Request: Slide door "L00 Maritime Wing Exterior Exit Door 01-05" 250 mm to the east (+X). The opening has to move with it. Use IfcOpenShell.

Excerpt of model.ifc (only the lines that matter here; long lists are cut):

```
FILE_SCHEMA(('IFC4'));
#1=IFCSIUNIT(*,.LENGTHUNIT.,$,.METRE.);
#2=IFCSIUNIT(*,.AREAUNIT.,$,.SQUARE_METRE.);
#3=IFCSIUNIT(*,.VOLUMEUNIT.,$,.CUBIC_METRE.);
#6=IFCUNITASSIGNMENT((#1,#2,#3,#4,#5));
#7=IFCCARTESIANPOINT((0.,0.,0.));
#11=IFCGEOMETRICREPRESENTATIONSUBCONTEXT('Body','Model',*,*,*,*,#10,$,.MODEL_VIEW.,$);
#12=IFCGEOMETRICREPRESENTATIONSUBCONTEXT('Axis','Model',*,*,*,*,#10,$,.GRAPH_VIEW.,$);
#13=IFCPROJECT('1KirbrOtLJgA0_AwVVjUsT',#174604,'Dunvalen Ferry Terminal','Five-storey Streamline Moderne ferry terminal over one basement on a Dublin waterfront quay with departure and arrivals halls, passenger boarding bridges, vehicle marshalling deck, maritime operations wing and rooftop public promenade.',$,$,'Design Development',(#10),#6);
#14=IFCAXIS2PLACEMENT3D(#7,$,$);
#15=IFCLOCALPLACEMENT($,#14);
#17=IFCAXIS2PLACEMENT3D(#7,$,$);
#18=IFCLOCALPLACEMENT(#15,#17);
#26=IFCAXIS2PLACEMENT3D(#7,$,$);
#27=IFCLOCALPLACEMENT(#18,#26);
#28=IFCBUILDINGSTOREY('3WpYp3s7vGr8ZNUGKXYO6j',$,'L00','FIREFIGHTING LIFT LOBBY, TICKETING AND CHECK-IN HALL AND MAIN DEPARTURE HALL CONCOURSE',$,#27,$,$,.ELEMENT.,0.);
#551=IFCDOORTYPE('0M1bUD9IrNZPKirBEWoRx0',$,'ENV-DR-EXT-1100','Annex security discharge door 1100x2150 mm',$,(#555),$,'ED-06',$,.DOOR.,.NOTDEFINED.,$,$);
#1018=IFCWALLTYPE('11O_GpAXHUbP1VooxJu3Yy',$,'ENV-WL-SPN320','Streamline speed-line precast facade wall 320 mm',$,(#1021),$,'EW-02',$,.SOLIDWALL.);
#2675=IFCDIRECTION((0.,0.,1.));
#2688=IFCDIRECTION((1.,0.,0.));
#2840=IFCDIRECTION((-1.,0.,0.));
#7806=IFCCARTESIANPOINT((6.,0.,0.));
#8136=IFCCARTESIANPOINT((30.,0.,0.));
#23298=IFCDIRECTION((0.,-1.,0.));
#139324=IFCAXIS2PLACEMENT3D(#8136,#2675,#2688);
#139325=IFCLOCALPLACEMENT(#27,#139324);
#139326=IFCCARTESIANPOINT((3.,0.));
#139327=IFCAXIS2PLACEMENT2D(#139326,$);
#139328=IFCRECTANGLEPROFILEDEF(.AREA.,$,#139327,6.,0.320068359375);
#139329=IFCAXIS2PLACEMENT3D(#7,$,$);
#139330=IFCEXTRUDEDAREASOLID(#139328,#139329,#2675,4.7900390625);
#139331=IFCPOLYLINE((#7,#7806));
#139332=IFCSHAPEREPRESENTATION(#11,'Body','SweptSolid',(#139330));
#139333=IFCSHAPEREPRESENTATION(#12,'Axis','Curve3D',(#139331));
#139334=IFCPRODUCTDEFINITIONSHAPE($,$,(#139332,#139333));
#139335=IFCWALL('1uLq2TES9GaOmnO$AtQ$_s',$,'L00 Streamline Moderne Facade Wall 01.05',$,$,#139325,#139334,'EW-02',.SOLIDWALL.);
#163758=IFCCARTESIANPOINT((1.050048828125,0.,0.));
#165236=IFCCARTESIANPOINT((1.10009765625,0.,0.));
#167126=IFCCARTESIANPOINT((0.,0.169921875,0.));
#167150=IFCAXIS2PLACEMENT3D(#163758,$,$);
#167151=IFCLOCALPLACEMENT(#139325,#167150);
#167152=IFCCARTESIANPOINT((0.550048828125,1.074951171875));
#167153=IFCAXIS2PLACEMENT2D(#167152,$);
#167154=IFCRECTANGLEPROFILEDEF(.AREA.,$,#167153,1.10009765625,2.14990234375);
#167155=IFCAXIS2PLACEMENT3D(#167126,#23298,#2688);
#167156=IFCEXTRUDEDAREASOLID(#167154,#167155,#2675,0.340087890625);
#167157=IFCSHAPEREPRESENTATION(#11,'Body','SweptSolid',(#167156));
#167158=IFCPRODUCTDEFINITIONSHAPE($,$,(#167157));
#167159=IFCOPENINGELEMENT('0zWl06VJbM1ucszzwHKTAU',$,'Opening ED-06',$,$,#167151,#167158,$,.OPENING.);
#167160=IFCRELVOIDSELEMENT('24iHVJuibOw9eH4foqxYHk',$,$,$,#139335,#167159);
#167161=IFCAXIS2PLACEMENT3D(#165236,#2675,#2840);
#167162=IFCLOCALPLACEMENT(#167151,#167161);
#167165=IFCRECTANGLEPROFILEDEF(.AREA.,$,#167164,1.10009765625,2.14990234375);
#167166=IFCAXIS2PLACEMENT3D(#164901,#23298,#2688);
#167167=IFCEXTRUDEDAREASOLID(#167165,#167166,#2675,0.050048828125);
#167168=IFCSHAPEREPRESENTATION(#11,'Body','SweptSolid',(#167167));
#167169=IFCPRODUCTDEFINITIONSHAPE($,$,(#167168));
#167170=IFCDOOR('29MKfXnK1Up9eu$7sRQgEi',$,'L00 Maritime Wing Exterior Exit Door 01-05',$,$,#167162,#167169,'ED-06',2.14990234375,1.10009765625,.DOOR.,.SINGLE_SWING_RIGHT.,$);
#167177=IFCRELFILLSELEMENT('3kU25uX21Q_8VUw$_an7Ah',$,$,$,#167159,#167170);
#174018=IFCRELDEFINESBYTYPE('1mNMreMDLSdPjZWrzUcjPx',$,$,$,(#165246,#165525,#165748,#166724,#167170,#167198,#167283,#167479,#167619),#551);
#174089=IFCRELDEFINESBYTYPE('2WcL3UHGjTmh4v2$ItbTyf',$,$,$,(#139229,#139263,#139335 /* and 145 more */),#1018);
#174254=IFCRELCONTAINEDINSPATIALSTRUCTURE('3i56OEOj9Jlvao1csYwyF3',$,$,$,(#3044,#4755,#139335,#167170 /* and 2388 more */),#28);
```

```python
import ifcopenshell
import ifcopenshell.api.geometry
import ifcopenshell.util.placement
import ifcopenshell.util.unit

model = ifcopenshell.open("model.ifc")
unit_scale = ifcopenshell.util.unit.calculate_unit_scale(model)

door = model.by_guid("29MKfXnK1Up9eu$7sRQgEi")
opening = door.FillsVoids[0].RelatingOpeningElement
wall = opening.VoidsElements[0].RelatingBuildingElement

wall_matrix = ifcopenshell.util.placement.get_local_placement(wall.ObjectPlacement)
shift = wall_matrix[:3, 0] * 0.25 / unit_scale
before = ifcopenshell.util.placement.get_local_placement(door.ObjectPlacement)[:3, 3].copy()

# The door is placed relative to its opening, so it follows when the opening moves.
matrix = ifcopenshell.util.placement.get_local_placement(opening.ObjectPlacement)
matrix[:3, 3] += shift
ifcopenshell.api.geometry.edit_object_placement(
    model, product=opening, matrix=matrix, is_si=False, should_transform_children=True
)

after = ifcopenshell.util.placement.get_local_placement(door.ObjectPlacement)[:3, 3]
print("door moved by", (after - before).round(3) + 0.0)

model.write("model_rev.ifc")
```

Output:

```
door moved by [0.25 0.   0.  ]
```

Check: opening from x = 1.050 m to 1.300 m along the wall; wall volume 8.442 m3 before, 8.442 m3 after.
